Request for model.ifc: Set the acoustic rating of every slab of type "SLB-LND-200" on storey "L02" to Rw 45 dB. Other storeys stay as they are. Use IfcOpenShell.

First a look at what the model holds.

```python
import ifcopenshell
import ifcopenshell.util.element

model = ifcopenshell.open("model.ifc")
print(model.schema)
storey = next(s for s in model.by_type("IfcBuildingStorey") if s.Name == "L02")
slabs = [e for e in ifcopenshell.util.element.get_decomposition(storey) if e.is_a("IfcSlab")]
seen = {}
for e in slabs:
    element_type = ifcopenshell.util.element.get_type(e)
    key = (element_type.Name if element_type != e and element_type else None, ifcopenshell.util.element.get_pset(e, "Pset_SlabCommon", "AcousticRating"))
    seen[key] = seen.get(key, 0) + 1
for (name, value), count in sorted(seen.items(), key=str):
    print(count, "x", name, "|", value)
```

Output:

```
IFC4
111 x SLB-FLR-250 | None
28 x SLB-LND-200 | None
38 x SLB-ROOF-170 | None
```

```python
import ifcopenshell
import ifcopenshell.api.pset
import ifcopenshell.util.element

model = ifcopenshell.open("model.ifc")

storey = next(s for s in model.by_type("IfcBuildingStorey") if s.Name == "L02")
slabs = [e for e in ifcopenshell.util.element.get_decomposition(storey) if e.is_a("IfcSlab")]

count = 0
for e in slabs:
    element_type = ifcopenshell.util.element.get_type(e)
    if element_type in (None, e) or element_type.Name != "SLB-LND-200":
        continue
    # add_pset returns the element's existing set when there is one.
    pset = ifcopenshell.api.pset.add_pset(model, product=e, name="Pset_SlabCommon")
    ifcopenshell.api.pset.edit_pset(model, pset=pset, properties={"AcousticRating": "Rw 45 dB"})
    count += 1

print(count, "slabs updated")

model.write("model_v2.ifc")
```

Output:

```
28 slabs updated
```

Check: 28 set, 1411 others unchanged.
